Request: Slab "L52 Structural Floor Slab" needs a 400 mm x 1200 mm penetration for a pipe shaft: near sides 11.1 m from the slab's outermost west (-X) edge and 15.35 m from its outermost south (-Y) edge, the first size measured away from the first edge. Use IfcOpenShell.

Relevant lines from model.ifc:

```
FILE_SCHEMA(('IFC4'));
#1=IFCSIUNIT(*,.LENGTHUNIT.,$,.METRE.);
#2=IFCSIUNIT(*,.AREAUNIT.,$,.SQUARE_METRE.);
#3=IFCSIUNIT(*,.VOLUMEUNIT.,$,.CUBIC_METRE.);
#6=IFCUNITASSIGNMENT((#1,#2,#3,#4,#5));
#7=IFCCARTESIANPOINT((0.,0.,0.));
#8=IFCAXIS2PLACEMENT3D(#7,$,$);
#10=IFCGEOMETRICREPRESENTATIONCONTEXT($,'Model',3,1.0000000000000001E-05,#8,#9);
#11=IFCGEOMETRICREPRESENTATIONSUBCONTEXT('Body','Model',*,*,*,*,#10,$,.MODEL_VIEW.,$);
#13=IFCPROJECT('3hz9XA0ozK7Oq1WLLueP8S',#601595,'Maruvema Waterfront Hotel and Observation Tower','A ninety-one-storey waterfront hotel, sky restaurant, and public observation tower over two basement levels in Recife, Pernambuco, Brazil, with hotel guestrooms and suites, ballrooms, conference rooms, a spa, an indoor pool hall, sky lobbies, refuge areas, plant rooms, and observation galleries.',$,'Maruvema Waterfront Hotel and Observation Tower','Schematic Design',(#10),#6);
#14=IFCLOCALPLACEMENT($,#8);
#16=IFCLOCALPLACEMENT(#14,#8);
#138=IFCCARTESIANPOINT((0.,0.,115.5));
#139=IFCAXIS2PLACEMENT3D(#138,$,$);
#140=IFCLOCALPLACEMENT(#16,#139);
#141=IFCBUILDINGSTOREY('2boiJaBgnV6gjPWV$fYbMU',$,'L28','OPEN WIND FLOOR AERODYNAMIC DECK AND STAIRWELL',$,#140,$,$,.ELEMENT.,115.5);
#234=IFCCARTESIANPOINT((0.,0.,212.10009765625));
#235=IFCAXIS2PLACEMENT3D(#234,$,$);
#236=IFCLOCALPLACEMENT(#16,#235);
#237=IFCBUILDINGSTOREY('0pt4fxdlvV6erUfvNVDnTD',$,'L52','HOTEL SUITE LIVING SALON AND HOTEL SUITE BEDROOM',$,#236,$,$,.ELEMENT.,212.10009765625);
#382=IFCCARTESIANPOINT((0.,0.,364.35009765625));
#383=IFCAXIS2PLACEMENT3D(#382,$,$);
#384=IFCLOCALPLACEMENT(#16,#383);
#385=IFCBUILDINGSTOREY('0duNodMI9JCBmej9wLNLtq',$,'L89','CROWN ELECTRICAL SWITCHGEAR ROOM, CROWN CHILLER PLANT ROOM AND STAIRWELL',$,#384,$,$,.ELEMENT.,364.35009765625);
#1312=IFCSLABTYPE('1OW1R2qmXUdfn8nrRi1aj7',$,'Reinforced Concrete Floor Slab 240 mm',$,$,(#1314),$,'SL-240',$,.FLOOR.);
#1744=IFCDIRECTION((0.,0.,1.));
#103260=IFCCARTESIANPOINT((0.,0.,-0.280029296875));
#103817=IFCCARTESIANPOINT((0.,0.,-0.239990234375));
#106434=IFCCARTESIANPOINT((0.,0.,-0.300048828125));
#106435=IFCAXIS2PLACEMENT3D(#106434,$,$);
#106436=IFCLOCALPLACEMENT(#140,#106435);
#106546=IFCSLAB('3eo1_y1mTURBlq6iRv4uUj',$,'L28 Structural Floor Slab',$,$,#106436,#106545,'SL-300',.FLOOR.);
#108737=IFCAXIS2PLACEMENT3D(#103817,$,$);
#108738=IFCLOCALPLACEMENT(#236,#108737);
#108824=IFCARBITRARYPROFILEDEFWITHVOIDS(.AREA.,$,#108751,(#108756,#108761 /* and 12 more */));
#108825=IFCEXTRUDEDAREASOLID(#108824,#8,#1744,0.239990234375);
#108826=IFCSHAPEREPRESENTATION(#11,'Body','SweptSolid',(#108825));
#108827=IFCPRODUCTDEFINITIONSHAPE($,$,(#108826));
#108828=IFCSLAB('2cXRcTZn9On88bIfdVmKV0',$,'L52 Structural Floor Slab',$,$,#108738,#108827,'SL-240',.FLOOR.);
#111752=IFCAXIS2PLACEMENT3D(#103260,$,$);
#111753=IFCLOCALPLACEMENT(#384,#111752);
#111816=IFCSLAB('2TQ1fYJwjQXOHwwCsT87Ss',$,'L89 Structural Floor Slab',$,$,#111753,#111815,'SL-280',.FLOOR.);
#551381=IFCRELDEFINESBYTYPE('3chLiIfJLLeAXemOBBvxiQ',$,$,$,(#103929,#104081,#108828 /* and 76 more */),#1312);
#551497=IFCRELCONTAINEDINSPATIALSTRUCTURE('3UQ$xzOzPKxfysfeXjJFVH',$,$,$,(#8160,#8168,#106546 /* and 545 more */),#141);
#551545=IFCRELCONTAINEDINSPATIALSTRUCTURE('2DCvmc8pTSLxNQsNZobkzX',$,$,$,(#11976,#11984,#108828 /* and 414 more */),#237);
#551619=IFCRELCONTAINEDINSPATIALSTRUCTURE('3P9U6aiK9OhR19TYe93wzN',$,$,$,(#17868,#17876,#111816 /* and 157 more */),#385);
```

```python
import numpy as np
import ifcopenshell
import ifcopenshell.api.feature
import ifcopenshell.api.geometry
import ifcopenshell.api.root
import ifcopenshell.geom
import ifcopenshell.util.placement
import ifcopenshell.util.representation
import ifcopenshell.util.shape
import ifcopenshell.util.unit

model = ifcopenshell.open("model.ifc")
unit_scale = ifcopenshell.util.unit.calculate_unit_scale(model)
settings = ifcopenshell.geom.settings()


def volume(element):
    """Net volume in cubic metres, openings subtracted."""
    shape = ifcopenshell.geom.create_shape(settings, element)
    return ifcopenshell.util.shape.get_volume(shape.geometry)


slab = model.by_id(108828)
before = volume(slab)

# Extent in the slab's own axes, in metres. The edges named are its -X and -Y sides.
slab_shape = ifcopenshell.geom.create_shape(settings, slab)
vertices = ifcopenshell.util.shape.get_vertices(slab_shape.geometry)
x_min, y_min, bottom = vertices.min(axis=0)
top = vertices[:, 2].max()

opening = ifcopenshell.api.root.create_entity(model, ifc_class="IfcOpeningElement", name="Pipe shaft opening", predefined_type="OPENING")
context = ifcopenshell.util.representation.get_context(model, "Model", "Body", "MODEL_VIEW")
width, depth = 0.4, 1.2
outline = [(0.0, 0.0), (width, 0.0), (width, depth), (0.0, depth), (0.0, 0.0)]
# Overshoot both faces by 50 mm so the cut is clean.
shape = ifcopenshell.api.geometry.add_slab_representation(
    model, context=context, depth=top - bottom + 0.1, polyline=outline
)
ifcopenshell.api.geometry.assign_representation(model, product=opening, representation=shape)

matrix = ifcopenshell.util.placement.get_local_placement(slab.ObjectPlacement)
matrix[:, 3] = matrix @ np.append(np.array([x_min + 11.1, y_min + 15.35, bottom - 0.05]) / unit_scale, 1.0)
ifcopenshell.api.geometry.edit_object_placement(model, product=opening, matrix=matrix, is_si=False)
ifcopenshell.api.feature.add_feature(model, feature=opening, element=slab)

after = volume(slab)

print(f"slab volume {before:.3f} -> {after:.3f} m3")

model.write("model_updated.ifc")
```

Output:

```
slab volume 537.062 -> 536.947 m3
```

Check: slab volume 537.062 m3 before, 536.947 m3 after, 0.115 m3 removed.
